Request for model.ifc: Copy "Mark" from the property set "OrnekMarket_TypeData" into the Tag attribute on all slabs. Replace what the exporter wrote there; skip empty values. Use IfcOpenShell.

First a look at what the model holds.

```python
import ifcopenshell
import ifcopenshell.util.element

model = ifcopenshell.open("model.ifc")
print(model.schema)
slabs = model.by_type("IfcSlab")
print(len(slabs), "slabs")
for e in slabs[:8]:
    source = ifcopenshell.util.element.get_pset(e, "OrnekMarket_TypeData", "Mark")
    target = e.Tag
    print(e.id(), repr(source), repr(target), sep=" | ")
```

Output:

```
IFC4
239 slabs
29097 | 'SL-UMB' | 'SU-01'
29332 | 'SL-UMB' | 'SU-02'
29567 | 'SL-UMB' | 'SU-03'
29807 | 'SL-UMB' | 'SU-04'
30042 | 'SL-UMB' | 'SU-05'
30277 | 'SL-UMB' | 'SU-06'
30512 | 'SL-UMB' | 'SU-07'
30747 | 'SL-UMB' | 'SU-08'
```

```python
import ifcopenshell
import ifcopenshell.util.element

model = ifcopenshell.open("model.ifc")

count = 0
for e in model.by_type("IfcSlab"):
    value = ifcopenshell.util.element.get_pset(e, "OrnekMarket_TypeData", "Mark")
    current = e.Tag
    if not value or not value.strip() or current == value:
        continue
    e.Tag = value
    count += 1

print(count, "slabs updated")

model.write("model_edited.ifc")
```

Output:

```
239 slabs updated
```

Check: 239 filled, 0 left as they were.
